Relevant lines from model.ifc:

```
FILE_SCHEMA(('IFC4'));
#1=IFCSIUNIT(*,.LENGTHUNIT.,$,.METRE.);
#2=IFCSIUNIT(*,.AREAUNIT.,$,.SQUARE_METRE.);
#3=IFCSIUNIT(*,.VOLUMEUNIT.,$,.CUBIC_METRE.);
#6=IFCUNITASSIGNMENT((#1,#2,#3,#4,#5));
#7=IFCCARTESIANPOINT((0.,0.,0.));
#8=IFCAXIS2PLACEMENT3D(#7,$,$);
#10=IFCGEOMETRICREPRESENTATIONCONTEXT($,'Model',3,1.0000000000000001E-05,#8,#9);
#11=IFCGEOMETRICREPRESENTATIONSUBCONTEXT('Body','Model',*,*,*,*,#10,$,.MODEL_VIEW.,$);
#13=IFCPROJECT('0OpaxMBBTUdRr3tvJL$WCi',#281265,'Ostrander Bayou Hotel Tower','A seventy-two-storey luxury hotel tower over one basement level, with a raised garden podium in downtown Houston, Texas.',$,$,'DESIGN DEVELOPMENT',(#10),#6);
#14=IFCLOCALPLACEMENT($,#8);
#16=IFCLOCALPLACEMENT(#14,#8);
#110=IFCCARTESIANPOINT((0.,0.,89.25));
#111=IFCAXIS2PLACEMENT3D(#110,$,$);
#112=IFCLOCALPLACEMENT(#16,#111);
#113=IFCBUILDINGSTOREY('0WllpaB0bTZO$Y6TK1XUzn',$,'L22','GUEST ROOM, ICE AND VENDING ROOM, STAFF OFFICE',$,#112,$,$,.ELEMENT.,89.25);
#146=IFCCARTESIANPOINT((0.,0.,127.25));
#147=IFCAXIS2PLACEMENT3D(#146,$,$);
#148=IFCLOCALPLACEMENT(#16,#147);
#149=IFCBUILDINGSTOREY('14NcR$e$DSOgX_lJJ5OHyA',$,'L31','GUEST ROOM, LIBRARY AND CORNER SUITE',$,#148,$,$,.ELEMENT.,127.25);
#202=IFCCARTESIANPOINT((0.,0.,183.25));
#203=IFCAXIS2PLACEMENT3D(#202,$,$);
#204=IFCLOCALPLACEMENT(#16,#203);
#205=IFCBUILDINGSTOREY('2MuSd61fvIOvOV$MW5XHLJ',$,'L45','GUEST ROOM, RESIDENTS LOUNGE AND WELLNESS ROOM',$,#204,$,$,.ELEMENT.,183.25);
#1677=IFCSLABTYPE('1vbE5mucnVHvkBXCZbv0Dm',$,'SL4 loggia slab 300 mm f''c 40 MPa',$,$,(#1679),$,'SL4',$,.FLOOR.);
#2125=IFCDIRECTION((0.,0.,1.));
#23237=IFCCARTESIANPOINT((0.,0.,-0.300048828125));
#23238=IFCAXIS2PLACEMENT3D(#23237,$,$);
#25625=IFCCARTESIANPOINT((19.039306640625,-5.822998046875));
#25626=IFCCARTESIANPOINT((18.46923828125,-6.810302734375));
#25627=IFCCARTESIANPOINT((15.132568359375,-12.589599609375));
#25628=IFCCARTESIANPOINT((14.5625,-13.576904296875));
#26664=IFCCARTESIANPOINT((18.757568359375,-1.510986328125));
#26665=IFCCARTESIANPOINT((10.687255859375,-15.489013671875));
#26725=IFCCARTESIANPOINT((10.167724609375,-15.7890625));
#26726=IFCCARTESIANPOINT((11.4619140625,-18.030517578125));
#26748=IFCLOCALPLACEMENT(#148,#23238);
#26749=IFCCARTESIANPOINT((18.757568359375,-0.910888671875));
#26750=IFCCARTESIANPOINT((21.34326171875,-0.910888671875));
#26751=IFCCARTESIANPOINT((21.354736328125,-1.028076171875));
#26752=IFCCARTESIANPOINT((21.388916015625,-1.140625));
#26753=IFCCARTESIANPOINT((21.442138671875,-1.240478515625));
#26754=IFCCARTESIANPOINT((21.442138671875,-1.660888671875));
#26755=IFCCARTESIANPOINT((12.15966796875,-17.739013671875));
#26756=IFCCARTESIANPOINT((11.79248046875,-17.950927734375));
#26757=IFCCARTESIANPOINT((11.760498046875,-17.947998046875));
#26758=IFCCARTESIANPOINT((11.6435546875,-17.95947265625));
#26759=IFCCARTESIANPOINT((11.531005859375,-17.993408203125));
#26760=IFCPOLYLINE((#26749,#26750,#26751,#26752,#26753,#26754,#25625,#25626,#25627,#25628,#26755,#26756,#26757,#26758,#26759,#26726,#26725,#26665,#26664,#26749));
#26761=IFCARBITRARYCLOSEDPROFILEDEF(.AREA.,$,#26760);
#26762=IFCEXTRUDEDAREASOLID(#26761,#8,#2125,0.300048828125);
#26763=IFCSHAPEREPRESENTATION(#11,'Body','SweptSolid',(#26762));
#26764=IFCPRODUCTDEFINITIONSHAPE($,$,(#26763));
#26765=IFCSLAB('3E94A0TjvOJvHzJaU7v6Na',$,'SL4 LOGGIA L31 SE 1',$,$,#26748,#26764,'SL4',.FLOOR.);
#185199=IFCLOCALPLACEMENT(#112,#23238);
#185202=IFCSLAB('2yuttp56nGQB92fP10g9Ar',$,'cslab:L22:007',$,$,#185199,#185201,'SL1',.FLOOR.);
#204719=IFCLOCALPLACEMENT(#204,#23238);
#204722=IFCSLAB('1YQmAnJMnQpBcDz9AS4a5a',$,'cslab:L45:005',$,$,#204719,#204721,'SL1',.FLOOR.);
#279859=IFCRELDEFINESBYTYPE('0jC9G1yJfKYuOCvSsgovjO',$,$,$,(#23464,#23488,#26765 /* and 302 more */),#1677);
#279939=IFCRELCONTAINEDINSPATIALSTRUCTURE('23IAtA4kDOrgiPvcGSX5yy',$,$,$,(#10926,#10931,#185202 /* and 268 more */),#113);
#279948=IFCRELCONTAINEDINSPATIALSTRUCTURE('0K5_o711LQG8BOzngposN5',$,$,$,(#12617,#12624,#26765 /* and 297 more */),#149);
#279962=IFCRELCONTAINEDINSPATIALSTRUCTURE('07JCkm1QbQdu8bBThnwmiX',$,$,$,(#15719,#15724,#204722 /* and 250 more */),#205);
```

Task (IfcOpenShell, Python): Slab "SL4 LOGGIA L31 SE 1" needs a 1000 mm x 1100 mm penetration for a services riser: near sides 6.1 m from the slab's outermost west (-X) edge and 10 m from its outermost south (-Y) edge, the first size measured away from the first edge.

```python
import numpy as np
import ifcopenshell
import ifcopenshell.api.feature
import ifcopenshell.api.geometry
import ifcopenshell.api.root
import ifcopenshell.geom
import ifcopenshell.util.placement
import ifcopenshell.util.representation
import ifcopenshell.util.shape
import ifcopenshell.util.unit

model = ifcopenshell.open("model.ifc")
unit_scale = ifcopenshell.util.unit.calculate_unit_scale(model)
settings = ifcopenshell.geom.settings()


def volume(element):
    """Net volume in cubic metres, openings subtracted."""
    shape = ifcopenshell.geom.create_shape(settings, element)
    return ifcopenshell.util.shape.get_volume(shape.geometry)


slab = model.by_guid("3E94A0TjvOJvHzJaU7v6Na")
before = volume(slab)

# Extent in the slab's own axes, in metres. The edges named are its -X and -Y sides.
slab_shape = ifcopenshell.geom.create_shape(settings, slab)
vertices = ifcopenshell.util.shape.get_vertices(slab_shape.geometry)
x_min, y_min, bottom = vertices.min(axis=0)
top = vertices[:, 2].max()

opening = ifcopenshell.api.root.create_entity(model, ifc_class="IfcOpeningElement", name="Services riser opening", predefined_type="OPENING")
context = ifcopenshell.util.representation.get_context(model, "Model", "Body", "MODEL_VIEW")
width, depth = 1, 1.1
outline = [(0.0, 0.0), (width, 0.0), (width, depth), (0.0, depth), (0.0, 0.0)]
# Overshoot both faces by 50 mm so the cut is clean.
shape = ifcopenshell.api.geometry.add_slab_representation(
    model, context=context, depth=top - bottom + 0.1, polyline=outline
)
ifcopenshell.api.geometry.assign_representation(model, product=opening, representation=shape)

matrix = ifcopenshell.util.placement.get_local_placement(slab.ObjectPlacement)
matrix[:, 3] = matrix @ np.append(np.array([x_min + 6.1, y_min + 10, bottom - 0.05]) / unit_scale, 1.0)
ifcopenshell.api.geometry.edit_object_placement(model, product=opening, matrix=matrix, is_si=False)
ifcopenshell.api.feature.add_feature(model, feature=opening, element=slab)

after = volume(slab)

print(f"slab volume {before:.3f} -> {after:.3f} m3")

model.write("model_rev.ifc")
```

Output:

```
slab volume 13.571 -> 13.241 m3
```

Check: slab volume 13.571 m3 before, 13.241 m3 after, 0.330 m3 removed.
